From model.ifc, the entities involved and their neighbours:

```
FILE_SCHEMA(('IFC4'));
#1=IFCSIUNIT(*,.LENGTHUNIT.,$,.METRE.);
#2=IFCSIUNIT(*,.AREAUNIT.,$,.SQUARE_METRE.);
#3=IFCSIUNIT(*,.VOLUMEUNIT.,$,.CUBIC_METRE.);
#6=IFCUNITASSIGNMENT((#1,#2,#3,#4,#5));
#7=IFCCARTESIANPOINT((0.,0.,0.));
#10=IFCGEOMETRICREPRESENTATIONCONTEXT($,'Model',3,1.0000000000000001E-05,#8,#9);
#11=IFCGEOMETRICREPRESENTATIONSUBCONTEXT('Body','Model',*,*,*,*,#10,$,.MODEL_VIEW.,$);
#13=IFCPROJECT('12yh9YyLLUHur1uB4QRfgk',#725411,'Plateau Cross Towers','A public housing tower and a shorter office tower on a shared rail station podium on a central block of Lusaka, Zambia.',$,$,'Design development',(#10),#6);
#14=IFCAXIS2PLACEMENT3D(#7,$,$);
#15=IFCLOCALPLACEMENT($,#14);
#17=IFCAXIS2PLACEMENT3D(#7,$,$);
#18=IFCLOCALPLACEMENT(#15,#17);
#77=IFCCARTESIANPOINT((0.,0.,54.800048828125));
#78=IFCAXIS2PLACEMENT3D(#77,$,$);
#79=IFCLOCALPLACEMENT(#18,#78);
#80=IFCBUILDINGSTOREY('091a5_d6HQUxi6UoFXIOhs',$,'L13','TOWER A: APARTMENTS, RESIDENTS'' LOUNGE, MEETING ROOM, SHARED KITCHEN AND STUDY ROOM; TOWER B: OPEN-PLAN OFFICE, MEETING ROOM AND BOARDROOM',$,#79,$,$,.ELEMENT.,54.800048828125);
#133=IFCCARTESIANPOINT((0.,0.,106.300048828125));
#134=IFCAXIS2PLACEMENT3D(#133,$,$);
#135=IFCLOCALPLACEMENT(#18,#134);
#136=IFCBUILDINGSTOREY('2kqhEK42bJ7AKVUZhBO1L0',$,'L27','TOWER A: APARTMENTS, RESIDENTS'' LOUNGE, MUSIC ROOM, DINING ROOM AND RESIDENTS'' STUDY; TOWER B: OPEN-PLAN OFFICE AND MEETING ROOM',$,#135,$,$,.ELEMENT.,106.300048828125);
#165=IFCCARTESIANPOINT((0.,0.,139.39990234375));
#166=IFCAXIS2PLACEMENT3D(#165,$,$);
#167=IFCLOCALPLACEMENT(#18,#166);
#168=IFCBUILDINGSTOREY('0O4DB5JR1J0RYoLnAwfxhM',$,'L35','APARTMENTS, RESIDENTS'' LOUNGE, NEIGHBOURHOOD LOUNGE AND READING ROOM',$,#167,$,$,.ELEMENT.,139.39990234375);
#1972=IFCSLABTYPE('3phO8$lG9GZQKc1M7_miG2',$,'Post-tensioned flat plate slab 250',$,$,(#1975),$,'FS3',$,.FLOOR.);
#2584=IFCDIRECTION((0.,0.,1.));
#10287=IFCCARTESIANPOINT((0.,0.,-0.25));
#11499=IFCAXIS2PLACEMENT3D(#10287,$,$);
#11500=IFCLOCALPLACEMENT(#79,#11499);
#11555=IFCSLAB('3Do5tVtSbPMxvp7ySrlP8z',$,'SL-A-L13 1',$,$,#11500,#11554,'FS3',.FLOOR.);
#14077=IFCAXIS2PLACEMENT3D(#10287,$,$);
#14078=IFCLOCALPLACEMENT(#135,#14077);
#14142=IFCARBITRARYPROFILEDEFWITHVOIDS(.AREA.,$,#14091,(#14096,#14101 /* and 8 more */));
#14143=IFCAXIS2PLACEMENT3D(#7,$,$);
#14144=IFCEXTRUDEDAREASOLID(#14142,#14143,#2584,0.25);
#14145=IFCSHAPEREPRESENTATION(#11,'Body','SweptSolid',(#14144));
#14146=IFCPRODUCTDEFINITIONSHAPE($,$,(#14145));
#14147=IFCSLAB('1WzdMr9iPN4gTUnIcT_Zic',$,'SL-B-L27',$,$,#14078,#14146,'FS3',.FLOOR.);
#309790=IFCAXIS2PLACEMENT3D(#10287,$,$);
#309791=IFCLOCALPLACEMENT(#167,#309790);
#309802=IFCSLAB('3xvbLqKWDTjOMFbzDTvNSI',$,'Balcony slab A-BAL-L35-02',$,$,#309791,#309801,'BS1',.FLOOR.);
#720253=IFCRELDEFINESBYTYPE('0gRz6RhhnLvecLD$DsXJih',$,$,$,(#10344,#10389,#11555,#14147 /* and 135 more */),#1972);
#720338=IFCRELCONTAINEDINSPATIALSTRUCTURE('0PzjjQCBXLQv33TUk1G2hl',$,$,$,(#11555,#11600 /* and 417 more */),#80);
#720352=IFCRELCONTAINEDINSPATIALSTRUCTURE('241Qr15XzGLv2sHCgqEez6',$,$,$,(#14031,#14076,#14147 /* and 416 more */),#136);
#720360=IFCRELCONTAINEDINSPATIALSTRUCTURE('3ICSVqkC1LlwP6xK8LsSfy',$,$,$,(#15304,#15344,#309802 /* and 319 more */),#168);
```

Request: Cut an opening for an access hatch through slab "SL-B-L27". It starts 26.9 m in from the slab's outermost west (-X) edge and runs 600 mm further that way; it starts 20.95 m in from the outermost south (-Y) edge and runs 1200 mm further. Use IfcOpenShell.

```python
import numpy as np
import ifcopenshell
import ifcopenshell.api.feature
import ifcopenshell.api.geometry
import ifcopenshell.api.root
import ifcopenshell.geom
import ifcopenshell.util.placement
import ifcopenshell.util.representation
import ifcopenshell.util.shape
import ifcopenshell.util.unit

model = ifcopenshell.open("model.ifc")
unit_scale = ifcopenshell.util.unit.calculate_unit_scale(model)
settings = ifcopenshell.geom.settings()


def volume(element):
    """Net volume in cubic metres, openings subtracted."""
    shape = ifcopenshell.geom.create_shape(settings, element)
    return ifcopenshell.util.shape.get_volume(shape.geometry)


slab = model.by_guid("1WzdMr9iPN4gTUnIcT_Zic")
before = volume(slab)

# Extent in the slab's own axes, in metres. The edges named are its -X and -Y sides.
slab_shape = ifcopenshell.geom.create_shape(settings, slab)
vertices = ifcopenshell.util.shape.get_vertices(slab_shape.geometry)
x_min, y_min, bottom = vertices.min(axis=0)
top = vertices[:, 2].max()

opening = ifcopenshell.api.root.create_entity(model, ifc_class="IfcOpeningElement", name="Access hatch opening", predefined_type="OPENING")
context = ifcopenshell.util.representation.get_context(model, "Model", "Body", "MODEL_VIEW")
width, depth = 0.6, 1.2
outline = [(0.0, 0.0), (width, 0.0), (width, depth), (0.0, depth), (0.0, 0.0)]
# Overshoot both faces by 50 mm so the cut is clean.
shape = ifcopenshell.api.geometry.add_slab_representation(
    model, context=context, depth=top - bottom + 0.1, polyline=outline
)
ifcopenshell.api.geometry.assign_representation(model, product=opening, representation=shape)

matrix = ifcopenshell.util.placement.get_local_placement(slab.ObjectPlacement)
matrix[:, 3] = matrix @ np.append(np.array([x_min + 26.9, y_min + 20.95, bottom - 0.05]) / unit_scale, 1.0)
ifcopenshell.api.geometry.edit_object_placement(model, product=opening, matrix=matrix, is_si=False)
ifcopenshell.api.feature.add_feature(model, feature=opening, element=slab)

after = volume(slab)

print(f"slab volume {before:.3f} -> {after:.3f} m3")

model.write("model_rev.ifc")
```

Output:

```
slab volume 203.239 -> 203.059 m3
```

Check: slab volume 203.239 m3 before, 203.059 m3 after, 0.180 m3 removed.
